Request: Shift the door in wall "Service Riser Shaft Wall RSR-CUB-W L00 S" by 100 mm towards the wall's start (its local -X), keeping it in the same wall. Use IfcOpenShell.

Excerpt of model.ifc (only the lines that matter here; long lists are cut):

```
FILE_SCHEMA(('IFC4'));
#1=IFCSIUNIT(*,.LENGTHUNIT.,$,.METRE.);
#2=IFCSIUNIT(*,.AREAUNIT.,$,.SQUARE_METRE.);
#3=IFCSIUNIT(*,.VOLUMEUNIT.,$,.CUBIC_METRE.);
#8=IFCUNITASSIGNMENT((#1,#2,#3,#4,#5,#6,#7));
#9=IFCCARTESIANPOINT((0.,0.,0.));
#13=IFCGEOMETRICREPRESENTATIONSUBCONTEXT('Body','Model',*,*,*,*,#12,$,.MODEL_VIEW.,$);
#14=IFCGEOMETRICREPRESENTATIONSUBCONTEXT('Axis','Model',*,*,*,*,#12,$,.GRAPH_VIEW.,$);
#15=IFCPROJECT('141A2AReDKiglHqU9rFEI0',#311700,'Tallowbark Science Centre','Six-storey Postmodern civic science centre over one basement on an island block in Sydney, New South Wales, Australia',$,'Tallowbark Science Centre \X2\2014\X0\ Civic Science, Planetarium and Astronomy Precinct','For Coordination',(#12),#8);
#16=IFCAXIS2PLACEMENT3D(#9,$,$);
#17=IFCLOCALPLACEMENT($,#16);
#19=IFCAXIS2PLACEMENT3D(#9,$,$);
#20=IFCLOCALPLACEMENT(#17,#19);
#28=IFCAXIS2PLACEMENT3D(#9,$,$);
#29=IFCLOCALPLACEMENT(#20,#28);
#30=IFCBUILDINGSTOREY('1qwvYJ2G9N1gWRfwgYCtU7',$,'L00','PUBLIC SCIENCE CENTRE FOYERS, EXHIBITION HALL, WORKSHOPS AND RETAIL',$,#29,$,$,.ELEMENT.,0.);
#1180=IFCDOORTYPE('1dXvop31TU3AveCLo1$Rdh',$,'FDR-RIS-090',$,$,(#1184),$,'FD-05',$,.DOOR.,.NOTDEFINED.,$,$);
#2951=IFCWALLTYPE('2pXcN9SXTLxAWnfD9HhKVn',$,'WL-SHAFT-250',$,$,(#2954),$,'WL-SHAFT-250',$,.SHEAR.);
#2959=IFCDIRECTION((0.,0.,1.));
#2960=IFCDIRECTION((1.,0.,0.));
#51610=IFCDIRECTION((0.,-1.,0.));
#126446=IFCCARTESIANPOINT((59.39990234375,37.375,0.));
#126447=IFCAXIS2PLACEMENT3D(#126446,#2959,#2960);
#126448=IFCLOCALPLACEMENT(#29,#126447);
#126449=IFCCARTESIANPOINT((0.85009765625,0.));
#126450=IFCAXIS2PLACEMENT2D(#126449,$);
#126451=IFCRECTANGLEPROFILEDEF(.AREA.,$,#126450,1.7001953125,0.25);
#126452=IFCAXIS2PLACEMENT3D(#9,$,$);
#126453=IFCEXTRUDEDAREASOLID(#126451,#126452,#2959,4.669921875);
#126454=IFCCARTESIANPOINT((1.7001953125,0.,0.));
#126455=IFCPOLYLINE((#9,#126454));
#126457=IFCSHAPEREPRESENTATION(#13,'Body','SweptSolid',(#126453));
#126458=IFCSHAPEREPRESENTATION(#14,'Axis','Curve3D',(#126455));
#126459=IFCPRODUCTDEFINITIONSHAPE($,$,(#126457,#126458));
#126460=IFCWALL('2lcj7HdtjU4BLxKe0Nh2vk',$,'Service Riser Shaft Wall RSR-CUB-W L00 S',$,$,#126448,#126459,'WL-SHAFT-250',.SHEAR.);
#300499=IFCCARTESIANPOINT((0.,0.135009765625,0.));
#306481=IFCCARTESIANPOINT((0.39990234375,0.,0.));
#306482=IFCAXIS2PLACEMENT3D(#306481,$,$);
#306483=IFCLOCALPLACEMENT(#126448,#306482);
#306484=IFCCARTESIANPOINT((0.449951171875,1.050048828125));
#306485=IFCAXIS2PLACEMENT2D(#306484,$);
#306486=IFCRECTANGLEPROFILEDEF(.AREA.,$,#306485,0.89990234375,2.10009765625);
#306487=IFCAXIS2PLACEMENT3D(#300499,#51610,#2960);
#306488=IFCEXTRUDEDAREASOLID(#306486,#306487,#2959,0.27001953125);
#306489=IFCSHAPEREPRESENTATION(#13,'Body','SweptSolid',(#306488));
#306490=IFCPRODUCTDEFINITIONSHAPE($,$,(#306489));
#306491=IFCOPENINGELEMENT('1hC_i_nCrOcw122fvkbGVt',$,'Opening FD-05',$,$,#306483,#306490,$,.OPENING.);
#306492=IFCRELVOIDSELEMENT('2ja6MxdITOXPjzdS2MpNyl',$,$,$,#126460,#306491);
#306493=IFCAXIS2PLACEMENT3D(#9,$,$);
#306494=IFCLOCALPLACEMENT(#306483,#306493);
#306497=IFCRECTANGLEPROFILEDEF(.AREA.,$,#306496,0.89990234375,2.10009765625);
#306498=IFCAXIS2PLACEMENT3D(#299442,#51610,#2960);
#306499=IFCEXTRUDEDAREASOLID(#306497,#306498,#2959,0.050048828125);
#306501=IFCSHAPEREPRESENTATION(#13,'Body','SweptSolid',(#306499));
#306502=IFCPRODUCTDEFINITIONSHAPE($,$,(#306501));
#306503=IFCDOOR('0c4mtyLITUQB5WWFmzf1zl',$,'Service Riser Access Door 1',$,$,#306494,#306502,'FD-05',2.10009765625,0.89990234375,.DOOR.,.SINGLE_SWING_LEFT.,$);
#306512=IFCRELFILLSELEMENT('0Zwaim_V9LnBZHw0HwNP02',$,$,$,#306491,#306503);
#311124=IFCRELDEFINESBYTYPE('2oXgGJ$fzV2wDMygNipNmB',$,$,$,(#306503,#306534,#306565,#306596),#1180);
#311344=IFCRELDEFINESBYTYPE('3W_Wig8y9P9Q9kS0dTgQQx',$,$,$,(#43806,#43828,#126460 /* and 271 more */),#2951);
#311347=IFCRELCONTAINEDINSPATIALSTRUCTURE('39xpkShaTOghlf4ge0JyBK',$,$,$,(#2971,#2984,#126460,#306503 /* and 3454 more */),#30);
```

```python
import ifcopenshell
import ifcopenshell.api.geometry
import ifcopenshell.util.placement
import ifcopenshell.util.unit

model = ifcopenshell.open("model.ifc")
unit_scale = ifcopenshell.util.unit.calculate_unit_scale(model)

door = model.by_id(306503)
opening = door.FillsVoids[0].RelatingOpeningElement
wall = opening.VoidsElements[0].RelatingBuildingElement

wall_matrix = ifcopenshell.util.placement.get_local_placement(wall.ObjectPlacement)
shift = wall_matrix[:3, 0] * -0.1 / unit_scale
before = ifcopenshell.util.placement.get_local_placement(door.ObjectPlacement)[:3, 3].copy()

# The door is placed relative to its opening, so it follows when the opening moves.
matrix = ifcopenshell.util.placement.get_local_placement(opening.ObjectPlacement)
matrix[:3, 3] += shift
ifcopenshell.api.geometry.edit_object_placement(
    model, product=opening, matrix=matrix, is_si=False, should_transform_children=True
)

after = ifcopenshell.util.placement.get_local_placement(door.ObjectPlacement)[:3, 3]
print("door moved by", (after - before).round(3) + 0.0)

model.write("model_rev.ifc")
```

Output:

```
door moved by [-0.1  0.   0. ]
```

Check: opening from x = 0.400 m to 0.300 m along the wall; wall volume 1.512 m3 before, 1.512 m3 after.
